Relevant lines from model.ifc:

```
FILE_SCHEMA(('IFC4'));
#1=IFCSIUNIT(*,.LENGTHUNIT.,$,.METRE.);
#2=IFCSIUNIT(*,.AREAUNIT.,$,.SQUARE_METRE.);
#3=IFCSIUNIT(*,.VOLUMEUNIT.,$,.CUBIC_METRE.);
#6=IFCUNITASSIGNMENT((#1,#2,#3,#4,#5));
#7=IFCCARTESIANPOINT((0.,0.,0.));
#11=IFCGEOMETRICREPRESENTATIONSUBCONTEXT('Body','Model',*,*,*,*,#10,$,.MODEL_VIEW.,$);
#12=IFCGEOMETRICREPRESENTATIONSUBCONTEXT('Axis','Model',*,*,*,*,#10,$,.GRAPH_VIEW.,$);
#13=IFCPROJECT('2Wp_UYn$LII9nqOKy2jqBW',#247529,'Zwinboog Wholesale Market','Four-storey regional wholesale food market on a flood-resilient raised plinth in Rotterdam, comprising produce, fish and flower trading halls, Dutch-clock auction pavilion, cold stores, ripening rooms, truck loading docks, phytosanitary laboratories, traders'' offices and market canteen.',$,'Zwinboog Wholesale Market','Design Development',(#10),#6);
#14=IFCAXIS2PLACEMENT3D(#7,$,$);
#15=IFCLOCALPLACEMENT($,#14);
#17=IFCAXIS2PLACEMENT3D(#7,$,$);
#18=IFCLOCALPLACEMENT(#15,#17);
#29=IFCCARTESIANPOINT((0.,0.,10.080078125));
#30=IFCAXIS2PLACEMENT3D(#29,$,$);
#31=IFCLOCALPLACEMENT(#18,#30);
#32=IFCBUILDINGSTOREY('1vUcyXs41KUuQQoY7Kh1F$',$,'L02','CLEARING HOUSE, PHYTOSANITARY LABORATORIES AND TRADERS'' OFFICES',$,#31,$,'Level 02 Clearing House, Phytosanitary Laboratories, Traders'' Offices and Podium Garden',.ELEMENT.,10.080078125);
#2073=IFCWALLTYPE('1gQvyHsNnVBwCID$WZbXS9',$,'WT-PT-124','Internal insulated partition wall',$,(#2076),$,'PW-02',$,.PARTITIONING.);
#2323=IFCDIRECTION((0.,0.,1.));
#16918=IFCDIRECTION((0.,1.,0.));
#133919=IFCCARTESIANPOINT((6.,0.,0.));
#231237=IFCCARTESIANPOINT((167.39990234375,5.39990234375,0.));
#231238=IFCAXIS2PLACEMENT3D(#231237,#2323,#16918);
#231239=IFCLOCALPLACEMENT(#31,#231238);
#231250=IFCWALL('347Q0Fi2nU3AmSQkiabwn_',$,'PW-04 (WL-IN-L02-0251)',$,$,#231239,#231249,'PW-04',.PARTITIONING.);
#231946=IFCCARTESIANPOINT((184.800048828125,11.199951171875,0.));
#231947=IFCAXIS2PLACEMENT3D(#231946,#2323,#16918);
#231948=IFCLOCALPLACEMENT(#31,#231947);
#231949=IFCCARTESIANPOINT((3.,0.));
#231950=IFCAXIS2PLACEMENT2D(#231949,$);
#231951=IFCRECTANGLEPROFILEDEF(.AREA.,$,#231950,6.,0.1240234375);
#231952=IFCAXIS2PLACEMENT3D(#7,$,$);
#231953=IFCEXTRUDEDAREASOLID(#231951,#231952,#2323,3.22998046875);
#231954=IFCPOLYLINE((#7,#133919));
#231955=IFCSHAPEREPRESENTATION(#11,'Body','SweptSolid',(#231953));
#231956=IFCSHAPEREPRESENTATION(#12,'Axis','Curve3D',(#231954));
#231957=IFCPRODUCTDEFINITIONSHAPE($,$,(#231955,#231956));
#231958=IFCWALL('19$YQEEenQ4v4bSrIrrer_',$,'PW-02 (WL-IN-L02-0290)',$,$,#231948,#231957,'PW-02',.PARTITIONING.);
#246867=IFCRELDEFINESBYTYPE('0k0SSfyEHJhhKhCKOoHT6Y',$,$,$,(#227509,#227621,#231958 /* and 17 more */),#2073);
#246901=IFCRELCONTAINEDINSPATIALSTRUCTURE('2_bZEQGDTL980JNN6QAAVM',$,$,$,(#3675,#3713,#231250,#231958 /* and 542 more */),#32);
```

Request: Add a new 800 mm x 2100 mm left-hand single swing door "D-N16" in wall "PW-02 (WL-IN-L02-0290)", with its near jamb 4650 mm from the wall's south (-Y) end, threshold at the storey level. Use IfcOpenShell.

```python
import numpy as np
import ifcopenshell
import ifcopenshell.api.feature
import ifcopenshell.api.geometry
import ifcopenshell.api.root
import ifcopenshell.api.spatial
import ifcopenshell.geom
import ifcopenshell.util.element
import ifcopenshell.util.placement
import ifcopenshell.util.representation
import ifcopenshell.util.shape
import ifcopenshell.util.unit

model = ifcopenshell.open("model.ifc")
unit_scale = ifcopenshell.util.unit.calculate_unit_scale(model)
settings = ifcopenshell.geom.settings()


def volume(element):
    """Net volume in cubic metres, openings subtracted."""
    shape = ifcopenshell.geom.create_shape(settings, element)
    return ifcopenshell.util.shape.get_volume(shape.geometry)


wall = model.by_guid("19$YQEEenQ4v4bSrIrrer_")
storey = ifcopenshell.util.element.get_container(wall, ifc_class="IfcBuildingStorey")
context = ifcopenshell.util.representation.get_context(model, "Model", "Body", "MODEL_VIEW")
before = volume(wall)

width, height, from_end, sill = 0.8, 2.1, 4.65, 0.0  # metres

# The wall runs along its own X axis, and the end named is its -X end.
wall_shape = ifcopenshell.geom.create_shape(settings, wall)
x, y, z = ifcopenshell.util.shape.get_vertices(wall_shape.geometry).T
start = x.min() + from_end
face, thickness = float(y.min()), float(y.max() - y.min())
wall_matrix = ifcopenshell.util.placement.get_local_placement(wall.ObjectPlacement)
level = ifcopenshell.util.placement.get_local_placement(storey.ObjectPlacement)[2, 3]


def in_wall(x, y):
    """Placement at x, y metres in the wall's axes, at sill height."""
    matrix = wall_matrix.copy()
    matrix[:, 3] = wall_matrix @ np.array([x / unit_scale, y / unit_scale, 0.0, 1.0])
    matrix[2, 3] = level + sill / unit_scale
    return matrix


# Opening: a box that overshoots both wall faces by 50 mm.
opening = ifcopenshell.api.root.create_entity(model, ifc_class="IfcOpeningElement", predefined_type="OPENING")
box = ifcopenshell.api.geometry.add_wall_representation(
    model, context=context, length=width, height=height, thickness=thickness + 0.1
)
ifcopenshell.api.geometry.assign_representation(model, product=opening, representation=box)
ifcopenshell.api.geometry.edit_object_placement(model, product=opening, matrix=in_wall(start, face - 0.05), is_si=False)
ifcopenshell.api.feature.add_feature(model, feature=opening, element=wall)

door = ifcopenshell.api.root.create_entity(model, ifc_class="IfcDoor", name="D-N16", predefined_type="DOOR")
door.OverallWidth, door.OverallHeight = width / unit_scale, height / unit_scale
door.OperationType = "SINGLE_SWING_LEFT"
body = ifcopenshell.api.geometry.add_door_representation(
    model,
    context=context,
    overall_width=door.OverallWidth,
    overall_height=door.OverallHeight,
    operation_type="SINGLE_SWING_LEFT",
    lining_properties={"LiningDepth": thickness / unit_scale, "ThresholdDepth": thickness / unit_scale},
)
ifcopenshell.api.geometry.assign_representation(model, product=door, representation=body)
ifcopenshell.api.spatial.assign_container(model, products=[door], relating_structure=storey)
ifcopenshell.api.feature.add_filling(model, opening=opening, element=door)

# The lining spans the wall, so the door starts at the wall face.
ifcopenshell.api.geometry.edit_object_placement(model, product=door, matrix=in_wall(start, face), is_si=False)

after = volume(wall)

print(f"wall volume {before:.3f} -> {after:.3f} m3")

model.write("model_updated.ifc")
```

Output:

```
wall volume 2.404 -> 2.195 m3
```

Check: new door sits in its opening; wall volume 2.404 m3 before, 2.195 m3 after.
